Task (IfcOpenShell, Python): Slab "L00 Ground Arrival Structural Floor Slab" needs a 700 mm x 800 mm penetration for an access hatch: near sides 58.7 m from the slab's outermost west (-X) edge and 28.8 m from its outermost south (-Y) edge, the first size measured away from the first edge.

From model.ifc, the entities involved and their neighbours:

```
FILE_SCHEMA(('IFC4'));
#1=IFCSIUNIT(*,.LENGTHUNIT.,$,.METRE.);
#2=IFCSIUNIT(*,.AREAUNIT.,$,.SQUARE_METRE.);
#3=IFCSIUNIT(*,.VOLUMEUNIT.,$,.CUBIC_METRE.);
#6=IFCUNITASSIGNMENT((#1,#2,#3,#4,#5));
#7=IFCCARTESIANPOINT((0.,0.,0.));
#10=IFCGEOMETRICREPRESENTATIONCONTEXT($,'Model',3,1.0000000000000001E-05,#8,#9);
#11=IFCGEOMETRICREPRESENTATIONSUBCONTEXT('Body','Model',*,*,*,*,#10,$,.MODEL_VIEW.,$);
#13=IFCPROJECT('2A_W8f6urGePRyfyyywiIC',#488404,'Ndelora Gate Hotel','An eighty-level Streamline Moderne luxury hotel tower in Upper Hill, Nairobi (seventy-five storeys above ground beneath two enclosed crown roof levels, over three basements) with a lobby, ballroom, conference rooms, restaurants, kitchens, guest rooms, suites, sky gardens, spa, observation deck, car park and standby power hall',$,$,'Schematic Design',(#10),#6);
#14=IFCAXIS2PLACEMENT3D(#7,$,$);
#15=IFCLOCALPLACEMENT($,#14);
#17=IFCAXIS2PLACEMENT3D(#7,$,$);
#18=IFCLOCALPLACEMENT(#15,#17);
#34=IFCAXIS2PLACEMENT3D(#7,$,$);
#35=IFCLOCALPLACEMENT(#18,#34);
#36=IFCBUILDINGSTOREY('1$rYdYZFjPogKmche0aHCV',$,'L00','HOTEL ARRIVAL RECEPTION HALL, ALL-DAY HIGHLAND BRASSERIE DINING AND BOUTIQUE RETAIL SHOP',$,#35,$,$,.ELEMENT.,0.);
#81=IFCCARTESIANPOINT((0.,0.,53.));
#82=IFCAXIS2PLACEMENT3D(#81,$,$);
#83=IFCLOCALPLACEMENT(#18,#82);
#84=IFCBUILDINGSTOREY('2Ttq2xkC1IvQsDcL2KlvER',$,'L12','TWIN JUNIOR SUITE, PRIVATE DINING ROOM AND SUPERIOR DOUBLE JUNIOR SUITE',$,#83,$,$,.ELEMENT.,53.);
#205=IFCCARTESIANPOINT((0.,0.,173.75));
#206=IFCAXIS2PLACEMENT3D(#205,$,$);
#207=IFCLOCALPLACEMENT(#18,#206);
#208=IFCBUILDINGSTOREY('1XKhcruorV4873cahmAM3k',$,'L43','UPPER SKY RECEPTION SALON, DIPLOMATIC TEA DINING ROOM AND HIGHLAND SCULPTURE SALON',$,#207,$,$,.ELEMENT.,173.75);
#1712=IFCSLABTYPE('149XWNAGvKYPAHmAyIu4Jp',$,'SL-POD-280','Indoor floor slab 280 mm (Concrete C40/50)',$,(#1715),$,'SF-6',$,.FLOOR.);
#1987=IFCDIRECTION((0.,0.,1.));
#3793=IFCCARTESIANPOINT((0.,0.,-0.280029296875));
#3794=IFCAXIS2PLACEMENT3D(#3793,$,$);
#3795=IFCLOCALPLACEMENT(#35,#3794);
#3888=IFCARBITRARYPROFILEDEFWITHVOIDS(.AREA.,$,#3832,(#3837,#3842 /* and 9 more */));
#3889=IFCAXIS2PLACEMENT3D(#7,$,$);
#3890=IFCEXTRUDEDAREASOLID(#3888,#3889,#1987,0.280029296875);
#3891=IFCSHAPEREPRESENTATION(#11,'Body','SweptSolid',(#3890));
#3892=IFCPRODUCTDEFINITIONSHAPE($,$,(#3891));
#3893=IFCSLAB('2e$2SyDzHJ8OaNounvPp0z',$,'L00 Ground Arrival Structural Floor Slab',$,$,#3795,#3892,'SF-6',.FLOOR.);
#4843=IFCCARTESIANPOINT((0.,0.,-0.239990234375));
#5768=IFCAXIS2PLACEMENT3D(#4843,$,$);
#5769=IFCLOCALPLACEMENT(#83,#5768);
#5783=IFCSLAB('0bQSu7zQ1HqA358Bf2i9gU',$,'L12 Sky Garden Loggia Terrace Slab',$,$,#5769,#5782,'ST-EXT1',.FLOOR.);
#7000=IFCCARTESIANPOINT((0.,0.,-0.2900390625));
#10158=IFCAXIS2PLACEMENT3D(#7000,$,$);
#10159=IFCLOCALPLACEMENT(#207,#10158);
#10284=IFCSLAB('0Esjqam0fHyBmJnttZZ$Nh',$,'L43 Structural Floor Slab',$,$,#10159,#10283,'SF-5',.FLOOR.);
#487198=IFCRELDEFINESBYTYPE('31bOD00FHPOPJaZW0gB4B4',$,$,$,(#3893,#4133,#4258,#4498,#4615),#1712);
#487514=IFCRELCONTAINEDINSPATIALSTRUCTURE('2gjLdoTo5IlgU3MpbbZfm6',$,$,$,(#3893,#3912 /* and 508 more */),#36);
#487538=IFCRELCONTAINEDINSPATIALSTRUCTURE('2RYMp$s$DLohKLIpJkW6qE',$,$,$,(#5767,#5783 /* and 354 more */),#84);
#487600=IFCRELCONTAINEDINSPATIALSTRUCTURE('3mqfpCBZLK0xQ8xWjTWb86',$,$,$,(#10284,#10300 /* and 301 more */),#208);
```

```python
import numpy as np
import ifcopenshell
import ifcopenshell.api.feature
import ifcopenshell.api.geometry
import ifcopenshell.api.root
import ifcopenshell.geom
import ifcopenshell.util.placement
import ifcopenshell.util.representation
import ifcopenshell.util.shape
import ifcopenshell.util.unit

model = ifcopenshell.open("model.ifc")
unit_scale = ifcopenshell.util.unit.calculate_unit_scale(model)
settings = ifcopenshell.geom.settings()


def volume(element):
    """Net volume in cubic metres, openings subtracted."""
    shape = ifcopenshell.geom.create_shape(settings, element)
    return ifcopenshell.util.shape.get_volume(shape.geometry)


slab = model.by_guid("2e$2SyDzHJ8OaNounvPp0z")
before = volume(slab)

# Extent in the slab's own axes, in metres. The edges named are its -X and -Y sides.
slab_shape = ifcopenshell.geom.create_shape(settings, slab)
vertices = ifcopenshell.util.shape.get_vertices(slab_shape.geometry)
x_min, y_min, bottom = vertices.min(axis=0)
top = vertices[:, 2].max()

opening = ifcopenshell.api.root.create_entity(model, ifc_class="IfcOpeningElement", name="Access hatch opening", predefined_type="OPENING")
context = ifcopenshell.util.representation.get_context(model, "Model", "Body", "MODEL_VIEW")
width, depth = 0.7, 0.8
outline = [(0.0, 0.0), (width, 0.0), (width, depth), (0.0, depth), (0.0, 0.0)]
# Overshoot both faces by 50 mm so the cut is clean.
shape = ifcopenshell.api.geometry.add_slab_representation(
    model, context=context, depth=top - bottom + 0.1, polyline=outline
)
ifcopenshell.api.geometry.assign_representation(model, product=opening, representation=shape)

matrix = ifcopenshell.util.placement.get_local_placement(slab.ObjectPlacement)
matrix[:, 3] = matrix @ np.append(np.array([x_min + 58.7, y_min + 28.8, bottom - 0.05]) / unit_scale, 1.0)
ifcopenshell.api.geometry.edit_object_placement(model, product=opening, matrix=matrix, is_si=False)
ifcopenshell.api.feature.add_feature(model, feature=opening, element=slab)

after = volume(slab)

print(f"slab volume {before:.3f} -> {after:.3f} m3")

model.write("model_rev.ifc")
```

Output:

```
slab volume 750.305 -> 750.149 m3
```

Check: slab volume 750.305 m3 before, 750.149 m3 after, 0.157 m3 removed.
